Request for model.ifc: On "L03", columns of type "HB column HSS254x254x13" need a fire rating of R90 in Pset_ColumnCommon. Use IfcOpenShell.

First a look at what the model holds.

```python
import ifcopenshell
import ifcopenshell.util.element

model = ifcopenshell.open("model.ifc")
print(model.schema)
storey = next(s for s in model.by_type("IfcBuildingStorey") if s.Name == "L03")
columns = [e for e in ifcopenshell.util.element.get_decomposition(storey) if e.is_a("IfcColumn")]
seen = {}
for e in columns:
    element_type = ifcopenshell.util.element.get_type(e)
    key = (element_type.Name if element_type != e and element_type else None, ifcopenshell.util.element.get_pset(e, "Pset_ColumnCommon", "FireRating"))
    seen[key] = seen.get(key, 0) + 1
for (name, value), count in sorted(seen.items(), key=str):
    print(count, "x", name, "|", value)
```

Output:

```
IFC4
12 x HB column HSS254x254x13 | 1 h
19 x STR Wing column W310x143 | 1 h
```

```python
import ifcopenshell
import ifcopenshell.api.pset
import ifcopenshell.util.element

model = ifcopenshell.open("model.ifc")

storey = next(s for s in model.by_type("IfcBuildingStorey") if s.Name == "L03")
columns = [e for e in ifcopenshell.util.element.get_decomposition(storey) if e.is_a("IfcColumn")]

count = 0
for e in columns:
    element_type = ifcopenshell.util.element.get_type(e)
    if element_type in (None, e) or element_type.Name != "HB column HSS254x254x13":
        continue
    # add_pset returns the element's existing set when there is one.
    pset = ifcopenshell.api.pset.add_pset(model, product=e, name="Pset_ColumnCommon")
    ifcopenshell.api.pset.edit_pset(model, pset=pset, properties={"FireRating": "R90"})
    count += 1

print(count, "columns updated")

model.write("model_rev.ifc")
```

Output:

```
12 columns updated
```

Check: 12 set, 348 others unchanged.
